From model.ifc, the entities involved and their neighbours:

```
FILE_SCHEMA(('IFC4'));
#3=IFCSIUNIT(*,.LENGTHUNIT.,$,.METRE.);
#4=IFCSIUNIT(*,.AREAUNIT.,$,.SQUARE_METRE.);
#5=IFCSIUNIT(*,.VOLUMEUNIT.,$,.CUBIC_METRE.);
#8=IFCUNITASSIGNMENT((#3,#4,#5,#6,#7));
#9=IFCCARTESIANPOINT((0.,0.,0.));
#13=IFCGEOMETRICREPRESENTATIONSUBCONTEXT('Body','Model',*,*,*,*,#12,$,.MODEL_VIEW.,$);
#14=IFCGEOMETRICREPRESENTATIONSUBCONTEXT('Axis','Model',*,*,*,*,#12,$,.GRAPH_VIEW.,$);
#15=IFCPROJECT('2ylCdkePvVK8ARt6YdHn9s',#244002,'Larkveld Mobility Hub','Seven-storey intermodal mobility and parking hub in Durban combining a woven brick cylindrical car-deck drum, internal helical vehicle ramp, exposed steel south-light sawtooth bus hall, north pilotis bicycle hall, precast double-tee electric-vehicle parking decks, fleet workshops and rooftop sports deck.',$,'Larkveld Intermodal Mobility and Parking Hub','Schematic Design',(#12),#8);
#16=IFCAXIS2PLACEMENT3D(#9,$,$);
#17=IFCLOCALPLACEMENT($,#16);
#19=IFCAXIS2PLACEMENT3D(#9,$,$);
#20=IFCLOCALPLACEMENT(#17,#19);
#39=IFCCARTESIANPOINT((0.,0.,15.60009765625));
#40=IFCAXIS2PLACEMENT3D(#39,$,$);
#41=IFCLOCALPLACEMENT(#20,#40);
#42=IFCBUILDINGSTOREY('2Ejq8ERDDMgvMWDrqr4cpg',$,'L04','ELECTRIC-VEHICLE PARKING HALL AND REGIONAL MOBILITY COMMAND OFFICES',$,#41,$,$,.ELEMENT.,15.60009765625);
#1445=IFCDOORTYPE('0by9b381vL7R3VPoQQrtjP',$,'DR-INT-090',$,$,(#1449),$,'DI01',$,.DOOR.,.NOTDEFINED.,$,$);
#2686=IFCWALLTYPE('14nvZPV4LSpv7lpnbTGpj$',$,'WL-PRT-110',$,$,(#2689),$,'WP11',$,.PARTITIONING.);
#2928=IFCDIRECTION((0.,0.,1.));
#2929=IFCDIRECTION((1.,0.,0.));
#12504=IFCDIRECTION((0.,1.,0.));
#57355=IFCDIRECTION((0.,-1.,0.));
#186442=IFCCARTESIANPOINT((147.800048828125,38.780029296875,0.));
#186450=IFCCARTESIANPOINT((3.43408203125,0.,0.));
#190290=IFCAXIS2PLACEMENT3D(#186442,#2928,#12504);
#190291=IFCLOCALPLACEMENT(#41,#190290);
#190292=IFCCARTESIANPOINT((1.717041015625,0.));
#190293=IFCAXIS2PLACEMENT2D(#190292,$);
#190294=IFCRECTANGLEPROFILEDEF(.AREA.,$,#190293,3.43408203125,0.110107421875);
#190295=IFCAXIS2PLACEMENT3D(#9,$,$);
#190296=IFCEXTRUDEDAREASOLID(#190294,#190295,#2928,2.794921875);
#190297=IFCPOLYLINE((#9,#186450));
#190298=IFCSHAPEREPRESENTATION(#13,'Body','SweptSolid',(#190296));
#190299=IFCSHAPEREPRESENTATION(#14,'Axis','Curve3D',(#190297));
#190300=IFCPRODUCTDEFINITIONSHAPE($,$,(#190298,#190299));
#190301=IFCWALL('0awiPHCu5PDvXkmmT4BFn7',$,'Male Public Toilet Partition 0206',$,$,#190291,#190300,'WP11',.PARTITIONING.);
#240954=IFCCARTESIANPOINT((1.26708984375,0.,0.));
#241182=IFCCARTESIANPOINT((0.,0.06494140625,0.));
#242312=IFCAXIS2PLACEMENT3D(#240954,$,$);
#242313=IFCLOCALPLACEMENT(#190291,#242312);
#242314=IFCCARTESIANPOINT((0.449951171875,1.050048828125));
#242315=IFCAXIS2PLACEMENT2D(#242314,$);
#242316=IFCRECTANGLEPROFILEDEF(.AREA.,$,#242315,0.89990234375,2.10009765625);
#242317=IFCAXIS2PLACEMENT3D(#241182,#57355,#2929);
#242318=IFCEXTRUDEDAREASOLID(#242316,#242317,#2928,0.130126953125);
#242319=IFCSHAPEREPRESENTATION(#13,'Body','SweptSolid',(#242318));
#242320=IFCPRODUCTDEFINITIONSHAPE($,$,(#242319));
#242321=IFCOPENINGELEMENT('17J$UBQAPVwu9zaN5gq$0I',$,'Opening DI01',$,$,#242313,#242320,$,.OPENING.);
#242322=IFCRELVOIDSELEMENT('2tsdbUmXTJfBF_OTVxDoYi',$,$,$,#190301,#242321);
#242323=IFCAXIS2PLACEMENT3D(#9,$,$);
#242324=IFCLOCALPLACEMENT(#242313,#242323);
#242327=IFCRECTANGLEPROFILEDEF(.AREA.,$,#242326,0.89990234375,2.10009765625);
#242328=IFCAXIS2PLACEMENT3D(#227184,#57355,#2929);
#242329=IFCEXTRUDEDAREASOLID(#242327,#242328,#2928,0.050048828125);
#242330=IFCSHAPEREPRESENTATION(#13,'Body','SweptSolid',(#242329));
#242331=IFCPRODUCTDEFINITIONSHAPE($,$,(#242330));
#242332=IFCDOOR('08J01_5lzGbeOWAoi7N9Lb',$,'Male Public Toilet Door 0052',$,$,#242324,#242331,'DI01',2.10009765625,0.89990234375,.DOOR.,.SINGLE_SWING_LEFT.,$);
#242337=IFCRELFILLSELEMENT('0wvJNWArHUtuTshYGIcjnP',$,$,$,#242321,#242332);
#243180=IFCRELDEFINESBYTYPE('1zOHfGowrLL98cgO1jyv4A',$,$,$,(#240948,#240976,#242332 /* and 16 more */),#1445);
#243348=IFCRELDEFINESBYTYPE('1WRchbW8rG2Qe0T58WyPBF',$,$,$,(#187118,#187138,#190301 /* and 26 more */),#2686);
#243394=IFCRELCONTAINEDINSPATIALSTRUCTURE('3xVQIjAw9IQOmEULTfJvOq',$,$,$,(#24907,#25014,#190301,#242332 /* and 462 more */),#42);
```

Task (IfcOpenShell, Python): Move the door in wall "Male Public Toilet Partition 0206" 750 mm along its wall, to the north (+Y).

```python
import ifcopenshell
import ifcopenshell.api.geometry
import ifcopenshell.util.placement

model = ifcopenshell.open("model.ifc")

door = model.by_id(242332)
opening = door.FillsVoids[0].RelatingOpeningElement
wall = opening.VoidsElements[0].RelatingBuildingElement

wall_matrix = ifcopenshell.util.placement.get_local_placement(wall.ObjectPlacement)
shift = wall_matrix[:3, 0] * 0.75
before = ifcopenshell.util.placement.get_local_placement(door.ObjectPlacement)[:3, 3].copy()

# The door is placed relative to its opening, so it follows when the opening moves.
matrix = ifcopenshell.util.placement.get_local_placement(opening.ObjectPlacement)
matrix[:3, 3] += shift
ifcopenshell.api.geometry.edit_object_placement(
    model, product=opening, matrix=matrix, is_si=False, should_transform_children=True
)

after = ifcopenshell.util.placement.get_local_placement(door.ObjectPlacement)[:3, 3]
print("door moved by", (after - before).round(3) + 0.0)

model.write("model_updated.ifc")
```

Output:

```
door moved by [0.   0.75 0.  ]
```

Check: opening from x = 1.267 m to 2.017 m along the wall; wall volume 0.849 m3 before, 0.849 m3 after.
